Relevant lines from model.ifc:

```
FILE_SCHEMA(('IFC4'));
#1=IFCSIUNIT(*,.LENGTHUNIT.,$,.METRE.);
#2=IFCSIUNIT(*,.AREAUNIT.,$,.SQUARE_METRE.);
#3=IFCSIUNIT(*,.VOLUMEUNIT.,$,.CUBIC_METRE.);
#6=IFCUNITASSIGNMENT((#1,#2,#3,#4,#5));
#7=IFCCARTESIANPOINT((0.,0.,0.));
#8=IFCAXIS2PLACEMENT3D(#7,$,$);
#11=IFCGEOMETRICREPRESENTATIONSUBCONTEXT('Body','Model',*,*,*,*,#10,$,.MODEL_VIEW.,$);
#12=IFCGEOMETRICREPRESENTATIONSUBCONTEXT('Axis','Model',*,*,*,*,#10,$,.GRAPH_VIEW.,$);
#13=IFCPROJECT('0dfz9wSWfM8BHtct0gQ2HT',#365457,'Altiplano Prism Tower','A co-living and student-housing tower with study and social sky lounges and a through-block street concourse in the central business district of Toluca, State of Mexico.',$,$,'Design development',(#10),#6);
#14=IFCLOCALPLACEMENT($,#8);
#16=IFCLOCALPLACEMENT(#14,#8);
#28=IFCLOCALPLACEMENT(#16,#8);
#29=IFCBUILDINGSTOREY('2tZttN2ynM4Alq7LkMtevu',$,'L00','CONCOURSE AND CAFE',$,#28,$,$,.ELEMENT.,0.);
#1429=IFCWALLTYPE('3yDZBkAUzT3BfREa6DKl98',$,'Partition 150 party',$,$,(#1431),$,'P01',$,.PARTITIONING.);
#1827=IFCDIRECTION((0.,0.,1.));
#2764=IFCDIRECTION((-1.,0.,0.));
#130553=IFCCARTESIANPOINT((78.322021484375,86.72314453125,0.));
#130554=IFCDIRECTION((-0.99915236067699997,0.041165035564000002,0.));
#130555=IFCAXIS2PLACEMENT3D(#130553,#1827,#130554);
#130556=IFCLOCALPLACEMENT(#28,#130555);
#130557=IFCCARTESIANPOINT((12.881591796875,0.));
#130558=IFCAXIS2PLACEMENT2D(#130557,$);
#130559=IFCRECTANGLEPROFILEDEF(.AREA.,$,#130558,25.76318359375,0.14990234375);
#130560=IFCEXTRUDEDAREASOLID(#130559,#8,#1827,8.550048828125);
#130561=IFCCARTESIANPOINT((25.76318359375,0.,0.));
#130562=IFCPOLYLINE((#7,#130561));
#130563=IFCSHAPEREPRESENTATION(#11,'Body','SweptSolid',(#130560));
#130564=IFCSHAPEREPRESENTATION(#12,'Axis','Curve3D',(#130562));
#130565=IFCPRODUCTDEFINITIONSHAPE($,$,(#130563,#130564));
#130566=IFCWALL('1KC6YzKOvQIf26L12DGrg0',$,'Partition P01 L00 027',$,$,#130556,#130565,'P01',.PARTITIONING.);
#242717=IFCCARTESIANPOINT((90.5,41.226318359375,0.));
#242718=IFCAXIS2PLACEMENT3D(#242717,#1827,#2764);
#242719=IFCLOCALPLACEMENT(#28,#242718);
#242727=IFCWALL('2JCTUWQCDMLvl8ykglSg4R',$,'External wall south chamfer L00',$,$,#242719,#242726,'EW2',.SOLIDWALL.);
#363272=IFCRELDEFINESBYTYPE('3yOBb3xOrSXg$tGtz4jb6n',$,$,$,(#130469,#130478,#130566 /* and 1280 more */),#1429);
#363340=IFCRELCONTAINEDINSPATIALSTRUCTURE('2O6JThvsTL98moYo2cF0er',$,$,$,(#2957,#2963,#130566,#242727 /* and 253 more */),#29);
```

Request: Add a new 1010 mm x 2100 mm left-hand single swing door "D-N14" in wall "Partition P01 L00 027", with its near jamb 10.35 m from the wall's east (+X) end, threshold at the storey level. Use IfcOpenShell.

```python
import numpy as np
import ifcopenshell
import ifcopenshell.api.feature
import ifcopenshell.api.geometry
import ifcopenshell.api.root
import ifcopenshell.api.spatial
import ifcopenshell.geom
import ifcopenshell.util.element
import ifcopenshell.util.placement
import ifcopenshell.util.representation
import ifcopenshell.util.shape
import ifcopenshell.util.unit

model = ifcopenshell.open("model.ifc")
unit_scale = ifcopenshell.util.unit.calculate_unit_scale(model)
settings = ifcopenshell.geom.settings()


def volume(element):
    """Net volume in cubic metres, openings subtracted."""
    shape = ifcopenshell.geom.create_shape(settings, element)
    return ifcopenshell.util.shape.get_volume(shape.geometry)


wall = model.by_guid("1KC6YzKOvQIf26L12DGrg0")
storey = ifcopenshell.util.element.get_container(wall, ifc_class="IfcBuildingStorey")
context = ifcopenshell.util.representation.get_context(model, "Model", "Body", "MODEL_VIEW")
before = volume(wall)

width, height, from_end, sill = 1.01, 2.1, 10.35, 0.0  # metres

# The wall runs along its own X axis, and the end named is its -X end.
wall_shape = ifcopenshell.geom.create_shape(settings, wall)
x, y, z = ifcopenshell.util.shape.get_vertices(wall_shape.geometry).T
start = x.min() + from_end
face, thickness = float(y.min()), float(y.max() - y.min())
wall_matrix = ifcopenshell.util.placement.get_local_placement(wall.ObjectPlacement)
level = ifcopenshell.util.placement.get_local_placement(storey.ObjectPlacement)[2, 3]


def in_wall(x, y):
    """Placement at x, y metres in the wall's axes, at sill height."""
    matrix = wall_matrix.copy()
    matrix[:, 3] = wall_matrix @ np.array([x / unit_scale, y / unit_scale, 0.0, 1.0])
    matrix[2, 3] = level + sill / unit_scale
    return matrix


# Opening: a box that overshoots both wall faces by 50 mm.
opening = ifcopenshell.api.root.create_entity(model, ifc_class="IfcOpeningElement", predefined_type="OPENING")
box = ifcopenshell.api.geometry.add_wall_representation(
    model, context=context, length=width, height=height, thickness=thickness + 0.1
)
ifcopenshell.api.geometry.assign_representation(model, product=opening, representation=box)
ifcopenshell.api.geometry.edit_object_placement(model, product=opening, matrix=in_wall(start, face - 0.05), is_si=False)
ifcopenshell.api.feature.add_feature(model, feature=opening, element=wall)

door = ifcopenshell.api.root.create_entity(model, ifc_class="IfcDoor", name="D-N14", predefined_type="DOOR")
door.OverallWidth, door.OverallHeight = width / unit_scale, height / unit_scale
door.OperationType = "SINGLE_SWING_LEFT"
body = ifcopenshell.api.geometry.add_door_representation(
    model,
    context=context,
    overall_width=door.OverallWidth,
    overall_height=door.OverallHeight,
    operation_type="SINGLE_SWING_LEFT",
    lining_properties={"LiningDepth": thickness / unit_scale, "ThresholdDepth": thickness / unit_scale},
)
ifcopenshell.api.geometry.assign_representation(model, product=door, representation=body)
ifcopenshell.api.spatial.assign_container(model, products=[door], relating_structure=storey)
ifcopenshell.api.feature.add_filling(model, opening=opening, element=door)

# The lining spans the wall, so the door starts at the wall face.
ifcopenshell.api.geometry.edit_object_placement(model, product=door, matrix=in_wall(start, face), is_si=False)

after = volume(wall)

print(f"wall volume {before:.3f} -> {after:.3f} m3")

model.write("model-out.ifc")
```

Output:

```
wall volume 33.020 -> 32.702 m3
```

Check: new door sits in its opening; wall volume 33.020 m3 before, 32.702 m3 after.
